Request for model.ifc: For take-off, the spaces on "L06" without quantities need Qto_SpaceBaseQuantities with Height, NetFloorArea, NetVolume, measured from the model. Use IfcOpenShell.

First a look at what the model holds.

```python
import ifcopenshell
import ifcopenshell.util.element
import ifcopenshell.util.unit

model = ifcopenshell.open("model.ifc")
print(model.schema)
for unit_type in ("LENGTHUNIT", "AREAUNIT", "VOLUMEUNIT"):
    print(unit_type, ifcopenshell.util.unit.calculate_unit_scale(model, unit_type))
storey = next(s for s in model.by_type("IfcBuildingStorey") if s.Name == "L06")
spaces = [e for e in ifcopenshell.util.element.get_decomposition(storey) if e.is_a("IfcSpace")]
for e in sorted(spaces, key=lambda e: e.id()):
    print(e.id(), e.is_a(), e.Name, list(ifcopenshell.util.element.get_psets(e, qtos_only=True)), sep=" | ")
```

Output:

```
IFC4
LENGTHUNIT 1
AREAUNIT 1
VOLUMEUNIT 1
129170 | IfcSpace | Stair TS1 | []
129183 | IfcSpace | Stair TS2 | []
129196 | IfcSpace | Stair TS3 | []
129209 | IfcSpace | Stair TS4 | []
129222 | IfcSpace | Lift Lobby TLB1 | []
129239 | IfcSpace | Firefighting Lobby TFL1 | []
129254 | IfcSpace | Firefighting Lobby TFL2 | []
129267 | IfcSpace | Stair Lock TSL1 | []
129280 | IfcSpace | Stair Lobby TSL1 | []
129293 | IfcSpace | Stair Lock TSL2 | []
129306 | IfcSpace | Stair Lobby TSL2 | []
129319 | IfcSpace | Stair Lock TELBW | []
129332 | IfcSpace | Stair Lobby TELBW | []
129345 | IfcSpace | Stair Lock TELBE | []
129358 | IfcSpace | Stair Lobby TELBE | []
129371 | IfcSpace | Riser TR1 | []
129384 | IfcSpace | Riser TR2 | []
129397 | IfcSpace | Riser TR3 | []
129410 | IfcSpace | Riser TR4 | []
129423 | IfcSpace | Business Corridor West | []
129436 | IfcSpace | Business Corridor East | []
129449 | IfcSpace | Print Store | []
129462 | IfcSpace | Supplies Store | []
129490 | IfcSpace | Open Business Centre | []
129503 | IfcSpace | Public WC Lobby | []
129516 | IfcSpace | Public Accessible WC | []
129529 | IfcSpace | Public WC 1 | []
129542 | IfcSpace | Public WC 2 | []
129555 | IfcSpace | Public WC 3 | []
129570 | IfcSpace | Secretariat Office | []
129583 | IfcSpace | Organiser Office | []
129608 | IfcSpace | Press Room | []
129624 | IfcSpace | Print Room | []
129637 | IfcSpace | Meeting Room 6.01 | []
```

```python
import ifcopenshell
import ifcopenshell.api.pset
import ifcopenshell.geom
import ifcopenshell.util.element
import ifcopenshell.util.shape
import ifcopenshell.util.unit

model = ifcopenshell.open("model.ifc")
unit_scale = ifcopenshell.util.unit.calculate_unit_scale(model)
area_scale = ifcopenshell.util.unit.calculate_unit_scale(model, "AREAUNIT")
volume_scale = ifcopenshell.util.unit.calculate_unit_scale(model, "VOLUMEUNIT")
settings = ifcopenshell.geom.settings()

storey = next(s for s in model.by_type("IfcBuildingStorey") if s.Name == "L06")
spaces = [e for e in ifcopenshell.util.element.get_decomposition(storey) if e.is_a("IfcSpace")]

for e in sorted(spaces, key=lambda e: e.id()):
    if ifcopenshell.util.element.get_psets(e, qtos_only=True, should_inherit=False):
        continue
    # Geometry comes back in metres, in the element's own axes.
    shape = ifcopenshell.geom.create_shape(settings, e)
    values = {
        "Height": ifcopenshell.util.shape.get_z(shape.geometry) / unit_scale,
        "NetFloorArea": ifcopenshell.util.shape.get_footprint_area(shape.geometry) / area_scale,
        "NetVolume": ifcopenshell.util.shape.get_volume(shape.geometry) / volume_scale,
    }
    qto = ifcopenshell.api.pset.add_qto(model, product=e, name="Qto_SpaceBaseQuantities")
    ifcopenshell.api.pset.edit_qto(model, qto=qto, properties=values)
    print(e.id(), {k: round(v, 3) for k, v in values.items()})

model.write("model_rev.ifc")
```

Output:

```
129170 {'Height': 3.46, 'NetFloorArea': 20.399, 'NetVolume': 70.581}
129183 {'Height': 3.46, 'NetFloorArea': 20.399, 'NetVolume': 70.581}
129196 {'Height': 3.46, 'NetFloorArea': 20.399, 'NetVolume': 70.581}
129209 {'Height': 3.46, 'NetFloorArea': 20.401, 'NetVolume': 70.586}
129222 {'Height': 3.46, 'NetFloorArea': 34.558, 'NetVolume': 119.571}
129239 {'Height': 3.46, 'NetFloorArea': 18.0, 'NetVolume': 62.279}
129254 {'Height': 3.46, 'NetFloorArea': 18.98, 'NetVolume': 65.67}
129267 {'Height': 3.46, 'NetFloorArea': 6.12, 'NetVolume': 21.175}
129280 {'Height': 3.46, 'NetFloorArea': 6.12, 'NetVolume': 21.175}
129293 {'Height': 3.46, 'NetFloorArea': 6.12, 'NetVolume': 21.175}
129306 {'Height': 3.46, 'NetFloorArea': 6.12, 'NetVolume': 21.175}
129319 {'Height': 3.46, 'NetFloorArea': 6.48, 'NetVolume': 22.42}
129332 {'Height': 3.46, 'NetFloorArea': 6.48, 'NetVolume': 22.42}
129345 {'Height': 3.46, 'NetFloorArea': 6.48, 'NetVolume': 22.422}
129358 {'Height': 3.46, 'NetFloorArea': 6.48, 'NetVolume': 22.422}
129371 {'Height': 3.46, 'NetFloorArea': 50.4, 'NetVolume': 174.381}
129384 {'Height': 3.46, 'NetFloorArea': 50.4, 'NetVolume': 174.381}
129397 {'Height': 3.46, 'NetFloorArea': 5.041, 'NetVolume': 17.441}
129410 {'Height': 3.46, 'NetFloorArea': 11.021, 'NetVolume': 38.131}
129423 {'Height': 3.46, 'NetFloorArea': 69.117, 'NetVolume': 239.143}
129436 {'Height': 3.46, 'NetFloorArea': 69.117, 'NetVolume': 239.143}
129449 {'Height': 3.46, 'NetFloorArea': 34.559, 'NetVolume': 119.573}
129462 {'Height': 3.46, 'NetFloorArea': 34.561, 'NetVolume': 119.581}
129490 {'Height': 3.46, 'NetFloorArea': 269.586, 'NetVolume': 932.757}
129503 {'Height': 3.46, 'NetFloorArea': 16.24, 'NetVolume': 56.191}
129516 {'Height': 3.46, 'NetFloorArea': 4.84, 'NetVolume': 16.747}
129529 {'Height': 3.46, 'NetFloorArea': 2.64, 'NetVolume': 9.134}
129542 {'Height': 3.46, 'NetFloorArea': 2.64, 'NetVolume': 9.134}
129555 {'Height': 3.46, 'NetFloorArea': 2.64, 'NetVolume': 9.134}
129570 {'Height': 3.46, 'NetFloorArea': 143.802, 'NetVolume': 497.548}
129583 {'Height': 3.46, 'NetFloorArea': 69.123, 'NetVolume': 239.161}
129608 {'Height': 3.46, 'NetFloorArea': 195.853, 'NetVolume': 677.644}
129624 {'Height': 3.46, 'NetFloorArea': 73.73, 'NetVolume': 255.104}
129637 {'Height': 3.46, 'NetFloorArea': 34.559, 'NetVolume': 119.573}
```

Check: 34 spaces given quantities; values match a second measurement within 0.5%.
